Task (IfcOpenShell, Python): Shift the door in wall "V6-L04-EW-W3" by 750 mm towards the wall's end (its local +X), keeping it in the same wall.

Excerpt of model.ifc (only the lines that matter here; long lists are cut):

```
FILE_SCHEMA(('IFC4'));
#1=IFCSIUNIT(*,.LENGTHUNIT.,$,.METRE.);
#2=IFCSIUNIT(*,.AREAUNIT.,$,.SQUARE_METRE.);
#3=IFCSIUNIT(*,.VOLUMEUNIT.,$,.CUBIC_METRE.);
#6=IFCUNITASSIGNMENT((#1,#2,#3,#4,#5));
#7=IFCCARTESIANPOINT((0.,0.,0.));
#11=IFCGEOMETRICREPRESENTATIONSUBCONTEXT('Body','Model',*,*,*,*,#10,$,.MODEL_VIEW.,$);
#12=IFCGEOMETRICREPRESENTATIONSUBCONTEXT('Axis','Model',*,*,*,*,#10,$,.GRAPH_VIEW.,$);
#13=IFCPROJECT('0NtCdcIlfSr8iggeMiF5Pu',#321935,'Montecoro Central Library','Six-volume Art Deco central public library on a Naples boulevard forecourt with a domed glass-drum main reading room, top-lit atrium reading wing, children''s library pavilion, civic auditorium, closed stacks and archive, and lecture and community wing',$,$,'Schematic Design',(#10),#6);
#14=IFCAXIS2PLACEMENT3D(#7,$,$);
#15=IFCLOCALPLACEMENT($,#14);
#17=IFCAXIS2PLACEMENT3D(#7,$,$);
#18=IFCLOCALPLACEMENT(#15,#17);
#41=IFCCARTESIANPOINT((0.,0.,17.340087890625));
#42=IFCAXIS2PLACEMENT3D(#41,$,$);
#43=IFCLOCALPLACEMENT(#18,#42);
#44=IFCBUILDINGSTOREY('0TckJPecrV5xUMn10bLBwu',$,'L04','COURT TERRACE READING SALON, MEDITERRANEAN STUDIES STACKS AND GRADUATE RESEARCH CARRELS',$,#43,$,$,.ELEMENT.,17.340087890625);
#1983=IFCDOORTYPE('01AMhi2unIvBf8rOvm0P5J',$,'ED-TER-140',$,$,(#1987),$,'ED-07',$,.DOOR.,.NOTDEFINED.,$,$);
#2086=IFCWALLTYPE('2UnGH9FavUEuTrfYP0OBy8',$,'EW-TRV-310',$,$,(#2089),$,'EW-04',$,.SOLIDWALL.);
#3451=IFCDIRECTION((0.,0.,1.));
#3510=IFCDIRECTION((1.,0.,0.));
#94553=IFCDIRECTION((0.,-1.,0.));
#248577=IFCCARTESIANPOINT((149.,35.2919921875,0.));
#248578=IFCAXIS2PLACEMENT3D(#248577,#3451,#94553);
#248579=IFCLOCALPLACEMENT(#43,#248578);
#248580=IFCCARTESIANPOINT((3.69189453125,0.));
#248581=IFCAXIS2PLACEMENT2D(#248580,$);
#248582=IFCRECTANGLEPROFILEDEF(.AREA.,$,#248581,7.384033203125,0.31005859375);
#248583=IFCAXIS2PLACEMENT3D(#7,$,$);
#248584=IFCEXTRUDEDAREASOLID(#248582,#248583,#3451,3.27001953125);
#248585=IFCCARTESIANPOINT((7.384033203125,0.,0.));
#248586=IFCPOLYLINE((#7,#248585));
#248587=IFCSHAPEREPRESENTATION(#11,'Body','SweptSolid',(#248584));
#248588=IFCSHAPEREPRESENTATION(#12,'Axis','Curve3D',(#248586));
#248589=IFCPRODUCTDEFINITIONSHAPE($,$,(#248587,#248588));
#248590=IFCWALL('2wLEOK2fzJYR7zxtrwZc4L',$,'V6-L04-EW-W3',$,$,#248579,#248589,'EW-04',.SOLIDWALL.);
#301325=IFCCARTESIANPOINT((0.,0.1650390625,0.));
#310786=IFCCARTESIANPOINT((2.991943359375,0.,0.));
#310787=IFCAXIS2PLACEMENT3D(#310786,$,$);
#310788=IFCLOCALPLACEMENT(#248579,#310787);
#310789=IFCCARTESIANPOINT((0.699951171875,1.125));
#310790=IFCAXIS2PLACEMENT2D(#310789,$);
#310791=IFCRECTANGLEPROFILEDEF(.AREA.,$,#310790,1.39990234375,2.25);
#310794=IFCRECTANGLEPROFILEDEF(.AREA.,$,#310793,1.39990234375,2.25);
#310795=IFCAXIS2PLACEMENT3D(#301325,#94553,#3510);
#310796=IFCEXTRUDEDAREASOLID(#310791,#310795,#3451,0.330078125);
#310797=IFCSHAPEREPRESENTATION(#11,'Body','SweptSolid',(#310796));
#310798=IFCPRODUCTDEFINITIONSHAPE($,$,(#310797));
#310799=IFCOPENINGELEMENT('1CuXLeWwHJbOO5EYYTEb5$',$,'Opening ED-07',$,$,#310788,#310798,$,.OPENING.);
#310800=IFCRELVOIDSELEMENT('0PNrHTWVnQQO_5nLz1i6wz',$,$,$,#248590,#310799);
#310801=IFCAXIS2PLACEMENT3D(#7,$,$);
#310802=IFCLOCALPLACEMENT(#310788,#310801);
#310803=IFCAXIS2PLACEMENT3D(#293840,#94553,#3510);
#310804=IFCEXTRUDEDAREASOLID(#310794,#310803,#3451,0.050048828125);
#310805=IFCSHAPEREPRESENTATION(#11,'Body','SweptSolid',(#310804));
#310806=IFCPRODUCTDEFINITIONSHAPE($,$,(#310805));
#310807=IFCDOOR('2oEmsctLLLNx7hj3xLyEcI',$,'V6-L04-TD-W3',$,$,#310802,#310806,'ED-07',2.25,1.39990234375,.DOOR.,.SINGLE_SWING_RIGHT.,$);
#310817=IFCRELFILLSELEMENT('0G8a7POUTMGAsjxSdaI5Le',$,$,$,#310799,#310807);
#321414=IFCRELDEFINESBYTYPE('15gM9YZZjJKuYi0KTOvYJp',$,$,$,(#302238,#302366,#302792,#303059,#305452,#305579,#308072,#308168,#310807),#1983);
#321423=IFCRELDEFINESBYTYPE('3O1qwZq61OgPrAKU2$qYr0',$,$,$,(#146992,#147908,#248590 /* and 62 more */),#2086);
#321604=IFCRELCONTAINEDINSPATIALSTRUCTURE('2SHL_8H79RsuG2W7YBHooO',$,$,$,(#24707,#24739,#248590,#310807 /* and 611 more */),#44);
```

```python
import ifcopenshell
import ifcopenshell.api.geometry
import ifcopenshell.util.placement
import ifcopenshell.util.unit

model = ifcopenshell.open("model.ifc")
unit_scale = ifcopenshell.util.unit.calculate_unit_scale(model)

door = model.by_guid("2oEmsctLLLNx7hj3xLyEcI")
opening = door.FillsVoids[0].RelatingOpeningElement
wall = opening.VoidsElements[0].RelatingBuildingElement

wall_matrix = ifcopenshell.util.placement.get_local_placement(wall.ObjectPlacement)
shift = wall_matrix[:3, 0] * 0.75 / unit_scale
before = ifcopenshell.util.placement.get_local_placement(door.ObjectPlacement)[:3, 3].copy()

# The door is placed relative to its opening, so it follows when the opening moves.
matrix = ifcopenshell.util.placement.get_local_placement(opening.ObjectPlacement)
matrix[:3, 3] += shift
ifcopenshell.api.geometry.edit_object_placement(
    model, product=opening, matrix=matrix, is_si=False, should_transform_children=True
)

after = ifcopenshell.util.placement.get_local_placement(door.ObjectPlacement)[:3, 3]
print("door moved by", (after - before).round(3) + 0.0)

model.write("model_v2.ifc")
```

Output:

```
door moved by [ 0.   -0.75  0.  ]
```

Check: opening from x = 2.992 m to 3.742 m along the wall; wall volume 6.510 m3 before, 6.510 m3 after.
